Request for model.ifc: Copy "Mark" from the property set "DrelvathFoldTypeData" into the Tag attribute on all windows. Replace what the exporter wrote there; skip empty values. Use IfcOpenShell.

First a look at what the model holds.

```python
import ifcopenshell
import ifcopenshell.util.element

model = ifcopenshell.open("model.ifc")
print(model.schema)
windows = model.by_type("IfcWindow")
print(len(windows), "windows")
for e in windows[:8]:
    source = ifcopenshell.util.element.get_pset(e, "DrelvathFoldTypeData", "Mark")
    target = e.Tag
    print(e.id(), repr(source), repr(target), sep=" | ")
```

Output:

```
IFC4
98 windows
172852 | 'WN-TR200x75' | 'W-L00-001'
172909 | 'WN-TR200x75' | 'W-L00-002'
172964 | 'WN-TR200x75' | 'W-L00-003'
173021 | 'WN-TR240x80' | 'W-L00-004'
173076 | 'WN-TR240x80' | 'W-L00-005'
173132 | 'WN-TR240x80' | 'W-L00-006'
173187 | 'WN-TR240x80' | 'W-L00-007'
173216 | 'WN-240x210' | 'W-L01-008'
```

```python
import ifcopenshell
import ifcopenshell.util.element

model = ifcopenshell.open("model.ifc")

count = 0
for e in model.by_type("IfcWindow"):
    value = ifcopenshell.util.element.get_pset(e, "DrelvathFoldTypeData", "Mark")
    current = e.Tag
    if not value or not value.strip() or current == value:
        continue
    e.Tag = value
    count += 1

print(count, "windows updated")

model.write("model_rev.ifc")
```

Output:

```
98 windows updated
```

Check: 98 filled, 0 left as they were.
